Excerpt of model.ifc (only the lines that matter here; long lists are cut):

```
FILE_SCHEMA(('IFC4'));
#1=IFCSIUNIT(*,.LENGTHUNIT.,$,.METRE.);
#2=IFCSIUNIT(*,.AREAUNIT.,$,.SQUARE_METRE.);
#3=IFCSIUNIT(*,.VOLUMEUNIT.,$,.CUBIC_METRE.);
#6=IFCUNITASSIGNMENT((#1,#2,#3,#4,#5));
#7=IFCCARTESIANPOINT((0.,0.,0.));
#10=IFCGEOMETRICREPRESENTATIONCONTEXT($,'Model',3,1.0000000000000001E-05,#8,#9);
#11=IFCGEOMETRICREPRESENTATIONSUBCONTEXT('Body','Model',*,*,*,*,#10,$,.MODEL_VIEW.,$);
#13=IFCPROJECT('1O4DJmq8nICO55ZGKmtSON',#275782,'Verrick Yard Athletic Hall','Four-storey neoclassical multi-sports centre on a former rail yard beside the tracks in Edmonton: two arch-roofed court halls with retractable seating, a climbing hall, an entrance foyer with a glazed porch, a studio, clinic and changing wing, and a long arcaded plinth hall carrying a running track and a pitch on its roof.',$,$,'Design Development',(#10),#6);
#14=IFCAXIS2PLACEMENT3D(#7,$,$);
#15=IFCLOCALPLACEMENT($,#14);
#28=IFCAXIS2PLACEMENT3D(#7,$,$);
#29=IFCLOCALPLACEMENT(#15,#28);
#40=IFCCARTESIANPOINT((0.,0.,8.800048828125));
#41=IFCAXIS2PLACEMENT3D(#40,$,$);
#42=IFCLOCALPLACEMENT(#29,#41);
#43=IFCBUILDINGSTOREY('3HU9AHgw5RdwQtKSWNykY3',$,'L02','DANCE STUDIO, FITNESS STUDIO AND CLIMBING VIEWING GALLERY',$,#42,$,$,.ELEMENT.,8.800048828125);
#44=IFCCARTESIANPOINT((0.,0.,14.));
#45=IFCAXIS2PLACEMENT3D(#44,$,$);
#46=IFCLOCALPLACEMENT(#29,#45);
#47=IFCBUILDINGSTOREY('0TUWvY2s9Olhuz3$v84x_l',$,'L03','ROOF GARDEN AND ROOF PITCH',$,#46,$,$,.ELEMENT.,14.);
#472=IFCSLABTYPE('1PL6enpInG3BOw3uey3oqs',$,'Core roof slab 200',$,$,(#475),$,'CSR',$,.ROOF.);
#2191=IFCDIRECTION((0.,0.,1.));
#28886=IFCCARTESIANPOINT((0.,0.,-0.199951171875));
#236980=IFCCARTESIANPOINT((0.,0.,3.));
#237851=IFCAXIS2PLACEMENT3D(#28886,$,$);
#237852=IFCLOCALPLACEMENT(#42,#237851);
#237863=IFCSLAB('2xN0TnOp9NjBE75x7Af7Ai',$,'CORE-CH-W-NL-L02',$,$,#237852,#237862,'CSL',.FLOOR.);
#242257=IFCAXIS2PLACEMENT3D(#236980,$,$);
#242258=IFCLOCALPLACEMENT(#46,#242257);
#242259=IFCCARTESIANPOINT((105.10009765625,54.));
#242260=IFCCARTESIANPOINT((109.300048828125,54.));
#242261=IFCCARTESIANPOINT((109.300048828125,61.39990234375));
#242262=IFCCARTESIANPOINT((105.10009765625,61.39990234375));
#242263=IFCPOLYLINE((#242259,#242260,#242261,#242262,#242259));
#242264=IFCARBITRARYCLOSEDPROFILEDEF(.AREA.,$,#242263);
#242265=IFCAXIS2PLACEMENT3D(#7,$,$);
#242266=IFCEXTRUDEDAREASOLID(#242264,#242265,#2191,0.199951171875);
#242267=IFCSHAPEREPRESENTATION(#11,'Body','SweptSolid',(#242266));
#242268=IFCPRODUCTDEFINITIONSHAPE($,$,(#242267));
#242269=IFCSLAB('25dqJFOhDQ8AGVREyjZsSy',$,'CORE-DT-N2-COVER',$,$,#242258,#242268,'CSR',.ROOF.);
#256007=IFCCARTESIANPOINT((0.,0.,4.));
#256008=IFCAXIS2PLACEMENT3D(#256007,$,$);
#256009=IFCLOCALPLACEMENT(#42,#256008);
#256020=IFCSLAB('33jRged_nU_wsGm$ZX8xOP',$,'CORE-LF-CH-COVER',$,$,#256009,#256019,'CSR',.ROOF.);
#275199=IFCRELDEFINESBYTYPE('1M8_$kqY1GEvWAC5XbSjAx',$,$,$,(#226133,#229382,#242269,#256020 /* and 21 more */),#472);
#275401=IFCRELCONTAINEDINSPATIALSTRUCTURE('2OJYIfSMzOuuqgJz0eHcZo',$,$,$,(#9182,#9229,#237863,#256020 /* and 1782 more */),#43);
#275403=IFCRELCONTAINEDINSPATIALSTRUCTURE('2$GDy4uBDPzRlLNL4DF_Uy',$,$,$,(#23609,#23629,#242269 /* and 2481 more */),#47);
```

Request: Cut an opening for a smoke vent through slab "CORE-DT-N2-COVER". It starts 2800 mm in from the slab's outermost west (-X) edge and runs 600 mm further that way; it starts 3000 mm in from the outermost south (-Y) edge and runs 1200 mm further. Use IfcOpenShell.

```python
import numpy as np
import ifcopenshell
import ifcopenshell.api.feature
import ifcopenshell.api.geometry
import ifcopenshell.api.root
import ifcopenshell.geom
import ifcopenshell.util.placement
import ifcopenshell.util.representation
import ifcopenshell.util.shape
import ifcopenshell.util.unit

model = ifcopenshell.open("model.ifc")
unit_scale = ifcopenshell.util.unit.calculate_unit_scale(model)
settings = ifcopenshell.geom.settings()


def volume(element):
    """Net volume in cubic metres, openings subtracted."""
    shape = ifcopenshell.geom.create_shape(settings, element)
    return ifcopenshell.util.shape.get_volume(shape.geometry)


slab = model.by_guid("25dqJFOhDQ8AGVREyjZsSy")
before = volume(slab)

# Extent in the slab's own axes, in metres. The edges named are its -X and -Y sides.
slab_shape = ifcopenshell.geom.create_shape(settings, slab)
vertices = ifcopenshell.util.shape.get_vertices(slab_shape.geometry)
x_min, y_min, bottom = vertices.min(axis=0)
top = vertices[:, 2].max()

opening = ifcopenshell.api.root.create_entity(model, ifc_class="IfcOpeningElement", name="Smoke vent opening", predefined_type="OPENING")
context = ifcopenshell.util.representation.get_context(model, "Model", "Body", "MODEL_VIEW")
width, depth = 0.6, 1.2
outline = [(0.0, 0.0), (width, 0.0), (width, depth), (0.0, depth), (0.0, 0.0)]
# Overshoot both faces by 50 mm so the cut is clean.
shape = ifcopenshell.api.geometry.add_slab_representation(
    model, context=context, depth=top - bottom + 0.1, polyline=outline
)
ifcopenshell.api.geometry.assign_representation(model, product=opening, representation=shape)

matrix = ifcopenshell.util.placement.get_local_placement(slab.ObjectPlacement)
matrix[:, 3] = matrix @ np.append(np.array([x_min + 2.8, y_min + 3, bottom - 0.05]) / unit_scale, 1.0)
ifcopenshell.api.geometry.edit_object_placement(model, product=opening, matrix=matrix, is_si=False)
ifcopenshell.api.feature.add_feature(model, feature=opening, element=slab)

after = volume(slab)

print(f"slab volume {before:.3f} -> {after:.3f} m3")

model.write("model_rev.ifc")
```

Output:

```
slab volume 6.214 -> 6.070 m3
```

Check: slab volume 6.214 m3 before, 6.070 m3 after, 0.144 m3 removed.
